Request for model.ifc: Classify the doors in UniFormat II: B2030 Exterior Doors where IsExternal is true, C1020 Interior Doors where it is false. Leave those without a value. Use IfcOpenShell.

First a look at what the model holds.

```python
import ifcopenshell
import ifcopenshell.util.element

model = ifcopenshell.open("model.ifc")
print(model.schema)
print("classifications:", [c.Name for c in model.by_type("IfcClassification")])
values = [ifcopenshell.util.element.get_pset(e, "Pset_DoorCommon", "IsExternal") for e in model.by_type("IfcDoor")]
for value in (True, False, None):
    print("IsExternal", value, values.count(value))
```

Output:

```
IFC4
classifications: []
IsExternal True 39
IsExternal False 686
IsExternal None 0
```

```python
import ifcopenshell
import ifcopenshell.api.classification
import ifcopenshell.util.element

model = ifcopenshell.open("model.ifc")

system = ifcopenshell.api.classification.add_classification(model, classification="UniFormat II")

doors = model.by_type("IfcDoor")
external = {e: ifcopenshell.util.element.get_pset(e, "Pset_DoorCommon", "IsExternal") for e in doors}
for flag, code, name in ((True, "B2030", "Exterior Doors"), (False, "C1020", "Interior Doors")):
    products = [e for e in doors if external[e] is flag]
    ifcopenshell.api.classification.add_reference(
        model, products=products, classification=system, identification=code, name=name
    )
    print(code, len(products))

model.write("model-out.ifc")
```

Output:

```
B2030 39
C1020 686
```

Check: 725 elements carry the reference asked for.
